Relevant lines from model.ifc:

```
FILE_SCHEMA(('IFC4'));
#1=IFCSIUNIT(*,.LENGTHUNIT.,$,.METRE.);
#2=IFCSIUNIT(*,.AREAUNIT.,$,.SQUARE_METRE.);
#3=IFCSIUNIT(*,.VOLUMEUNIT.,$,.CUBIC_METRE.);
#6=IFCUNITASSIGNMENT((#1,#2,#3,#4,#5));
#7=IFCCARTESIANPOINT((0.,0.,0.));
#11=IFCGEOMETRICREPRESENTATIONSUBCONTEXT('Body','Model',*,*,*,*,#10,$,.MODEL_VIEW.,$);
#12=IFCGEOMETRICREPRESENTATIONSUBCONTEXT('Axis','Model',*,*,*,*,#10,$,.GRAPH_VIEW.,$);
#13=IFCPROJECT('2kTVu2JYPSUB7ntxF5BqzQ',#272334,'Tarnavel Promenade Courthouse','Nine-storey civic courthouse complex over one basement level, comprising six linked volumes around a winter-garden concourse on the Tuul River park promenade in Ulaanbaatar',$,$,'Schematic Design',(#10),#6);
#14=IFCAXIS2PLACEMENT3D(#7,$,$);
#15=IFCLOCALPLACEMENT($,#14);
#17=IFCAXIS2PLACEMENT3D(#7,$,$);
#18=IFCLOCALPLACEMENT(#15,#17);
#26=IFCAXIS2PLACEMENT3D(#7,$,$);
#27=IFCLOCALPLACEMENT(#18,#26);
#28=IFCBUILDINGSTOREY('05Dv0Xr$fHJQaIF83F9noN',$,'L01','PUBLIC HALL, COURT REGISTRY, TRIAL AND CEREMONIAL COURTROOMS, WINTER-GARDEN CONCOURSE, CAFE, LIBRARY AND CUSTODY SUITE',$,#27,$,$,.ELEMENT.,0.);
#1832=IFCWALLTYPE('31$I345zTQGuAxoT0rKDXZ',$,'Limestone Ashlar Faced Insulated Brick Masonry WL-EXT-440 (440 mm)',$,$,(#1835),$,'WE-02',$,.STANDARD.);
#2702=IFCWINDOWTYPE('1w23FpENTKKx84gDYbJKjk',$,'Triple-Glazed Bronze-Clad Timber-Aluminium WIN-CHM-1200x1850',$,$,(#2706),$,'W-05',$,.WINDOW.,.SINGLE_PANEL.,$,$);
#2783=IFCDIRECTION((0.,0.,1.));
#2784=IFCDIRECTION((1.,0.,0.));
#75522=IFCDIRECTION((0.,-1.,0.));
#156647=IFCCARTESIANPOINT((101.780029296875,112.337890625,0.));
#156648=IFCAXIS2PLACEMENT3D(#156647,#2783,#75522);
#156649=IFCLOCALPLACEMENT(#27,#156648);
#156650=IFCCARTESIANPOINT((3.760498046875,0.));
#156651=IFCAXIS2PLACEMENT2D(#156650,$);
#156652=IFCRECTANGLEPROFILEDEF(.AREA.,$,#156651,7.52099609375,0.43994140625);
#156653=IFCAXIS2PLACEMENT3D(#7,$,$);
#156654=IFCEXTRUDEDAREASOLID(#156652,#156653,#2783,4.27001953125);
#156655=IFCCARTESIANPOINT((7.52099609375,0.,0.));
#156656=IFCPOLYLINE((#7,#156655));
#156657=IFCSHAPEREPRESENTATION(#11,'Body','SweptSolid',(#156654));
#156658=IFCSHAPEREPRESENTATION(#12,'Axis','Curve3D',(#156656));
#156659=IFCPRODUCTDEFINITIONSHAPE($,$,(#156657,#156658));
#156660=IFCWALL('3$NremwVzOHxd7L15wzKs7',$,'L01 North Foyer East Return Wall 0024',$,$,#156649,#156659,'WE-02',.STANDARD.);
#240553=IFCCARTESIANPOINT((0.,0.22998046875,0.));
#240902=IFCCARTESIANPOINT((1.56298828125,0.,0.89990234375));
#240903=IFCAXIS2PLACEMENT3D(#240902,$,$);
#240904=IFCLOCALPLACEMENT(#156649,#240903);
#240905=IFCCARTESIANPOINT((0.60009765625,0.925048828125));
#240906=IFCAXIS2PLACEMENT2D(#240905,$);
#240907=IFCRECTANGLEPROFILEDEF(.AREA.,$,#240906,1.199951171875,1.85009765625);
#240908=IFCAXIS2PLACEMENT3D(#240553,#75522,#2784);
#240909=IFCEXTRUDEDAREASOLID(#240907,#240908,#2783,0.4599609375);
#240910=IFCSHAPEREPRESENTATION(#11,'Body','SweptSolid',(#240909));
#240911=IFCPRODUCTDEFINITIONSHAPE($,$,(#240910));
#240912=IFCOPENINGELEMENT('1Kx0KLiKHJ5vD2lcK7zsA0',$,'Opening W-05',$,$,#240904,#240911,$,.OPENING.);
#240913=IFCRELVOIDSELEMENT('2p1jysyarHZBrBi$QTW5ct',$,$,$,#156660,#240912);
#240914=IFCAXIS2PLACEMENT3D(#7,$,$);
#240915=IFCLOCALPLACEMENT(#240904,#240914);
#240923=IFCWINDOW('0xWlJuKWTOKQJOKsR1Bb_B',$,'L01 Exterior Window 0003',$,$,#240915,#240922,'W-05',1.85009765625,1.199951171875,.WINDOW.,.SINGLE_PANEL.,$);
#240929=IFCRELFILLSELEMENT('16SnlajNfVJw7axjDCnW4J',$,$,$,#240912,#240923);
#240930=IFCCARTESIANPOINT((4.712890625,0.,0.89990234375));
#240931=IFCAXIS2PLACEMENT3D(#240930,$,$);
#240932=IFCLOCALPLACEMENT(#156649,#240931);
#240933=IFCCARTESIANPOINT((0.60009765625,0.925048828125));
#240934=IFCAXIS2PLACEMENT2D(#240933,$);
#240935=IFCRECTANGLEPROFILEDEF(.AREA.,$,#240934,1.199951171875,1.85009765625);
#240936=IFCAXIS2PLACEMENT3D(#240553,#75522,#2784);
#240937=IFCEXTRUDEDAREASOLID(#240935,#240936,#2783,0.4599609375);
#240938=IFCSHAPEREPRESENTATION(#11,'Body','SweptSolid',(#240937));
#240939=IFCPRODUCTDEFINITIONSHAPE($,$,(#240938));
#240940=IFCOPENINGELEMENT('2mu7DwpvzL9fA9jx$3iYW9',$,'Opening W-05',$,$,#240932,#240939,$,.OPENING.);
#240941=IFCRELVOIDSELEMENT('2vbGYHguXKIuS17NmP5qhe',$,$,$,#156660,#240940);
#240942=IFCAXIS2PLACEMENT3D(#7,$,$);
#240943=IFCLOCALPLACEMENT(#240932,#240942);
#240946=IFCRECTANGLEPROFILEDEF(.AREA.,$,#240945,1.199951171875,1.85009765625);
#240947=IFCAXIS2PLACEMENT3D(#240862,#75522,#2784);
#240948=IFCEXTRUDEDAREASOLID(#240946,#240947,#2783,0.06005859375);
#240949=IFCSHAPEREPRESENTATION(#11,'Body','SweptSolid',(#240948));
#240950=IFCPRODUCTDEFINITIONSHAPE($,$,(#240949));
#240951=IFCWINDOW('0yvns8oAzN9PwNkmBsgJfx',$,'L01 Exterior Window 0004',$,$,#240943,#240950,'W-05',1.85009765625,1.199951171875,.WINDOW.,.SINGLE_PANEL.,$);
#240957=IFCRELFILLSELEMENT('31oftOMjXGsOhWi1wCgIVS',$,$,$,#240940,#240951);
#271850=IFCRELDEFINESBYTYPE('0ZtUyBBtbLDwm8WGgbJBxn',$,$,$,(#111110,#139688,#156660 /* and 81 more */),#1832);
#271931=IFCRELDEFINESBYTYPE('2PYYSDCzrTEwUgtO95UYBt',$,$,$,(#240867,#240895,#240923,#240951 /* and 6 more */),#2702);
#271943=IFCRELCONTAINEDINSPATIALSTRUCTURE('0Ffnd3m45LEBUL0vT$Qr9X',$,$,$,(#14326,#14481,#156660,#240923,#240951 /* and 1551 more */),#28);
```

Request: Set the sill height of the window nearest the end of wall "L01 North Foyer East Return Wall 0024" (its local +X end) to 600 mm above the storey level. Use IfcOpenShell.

```python
import numpy as np
import ifcopenshell
import ifcopenshell.api.geometry
import ifcopenshell.geom
import ifcopenshell.util.element
import ifcopenshell.util.placement
import ifcopenshell.util.shape
import ifcopenshell.util.unit

model = ifcopenshell.open("model.ifc")
unit_scale = ifcopenshell.util.unit.calculate_unit_scale(model)

window = model.by_id(240951)
opening = window.FillsVoids[0].RelatingOpeningElement
storey = ifcopenshell.util.element.get_container(window, ifc_class="IfcBuildingStorey")
level = ifcopenshell.util.placement.get_local_placement(storey.ObjectPlacement)[2, 3]

# The opening's origin need not be at the sill, so measure its lowest point.
shape = ifcopenshell.geom.create_shape(ifcopenshell.geom.settings(), opening)
bottom = ifcopenshell.util.shape.get_shape_bottom_elevation(shape, shape.geometry) / unit_scale
dz = level + 0.6 - bottom

shift = np.array([0.0, 0.0, dz])
# The window is placed relative to its opening, so it follows when the opening moves.
matrix = ifcopenshell.util.placement.get_local_placement(opening.ObjectPlacement)
matrix[:3, 3] += shift
ifcopenshell.api.geometry.edit_object_placement(
    model, product=opening, matrix=matrix, is_si=False, should_transform_children=True
)

print(f"moved by {dz * unit_scale:+.3f} m")

model.write("model_updated.ifc")
```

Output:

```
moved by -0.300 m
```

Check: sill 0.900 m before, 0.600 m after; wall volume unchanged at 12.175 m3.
